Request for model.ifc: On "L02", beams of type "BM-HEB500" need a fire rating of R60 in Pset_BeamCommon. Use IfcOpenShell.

First a look at what the model holds.

```python
import ifcopenshell
import ifcopenshell.util.element

model = ifcopenshell.open("model.ifc")
print(model.schema)
storey = next(s for s in model.by_type("IfcBuildingStorey") if s.Name == "L02")
beams = [e for e in ifcopenshell.util.element.get_decomposition(storey) if e.is_a("IfcBeam")]
seen = {}
for e in beams:
    element_type = ifcopenshell.util.element.get_type(e)
    key = (element_type.Name if element_type != e and element_type else None, ifcopenshell.util.element.get_pset(e, "Pset_BeamCommon", "FireRating"))
    seen[key] = seen.get(key, 0) + 1
for (name, value), count in sorted(seen.items(), key=str):
    print(count, "x", name, "|", value)
```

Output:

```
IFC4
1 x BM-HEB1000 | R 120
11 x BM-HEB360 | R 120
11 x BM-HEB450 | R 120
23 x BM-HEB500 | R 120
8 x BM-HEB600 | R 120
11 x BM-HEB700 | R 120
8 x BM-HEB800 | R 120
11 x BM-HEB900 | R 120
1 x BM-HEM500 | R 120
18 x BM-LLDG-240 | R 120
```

```python
import ifcopenshell
import ifcopenshell.api.pset
import ifcopenshell.util.element

model = ifcopenshell.open("model.ifc")

storey = next(s for s in model.by_type("IfcBuildingStorey") if s.Name == "L02")
beams = [e for e in ifcopenshell.util.element.get_decomposition(storey) if e.is_a("IfcBeam")]

count = 0
for e in beams:
    element_type = ifcopenshell.util.element.get_type(e)
    if element_type in (None, e) or element_type.Name != "BM-HEB500":
        continue
    found = ifcopenshell.util.element.get_pset(e, "Pset_BeamCommon", should_inherit=False)
    if found:
        pset = model.by_id(found["id"])
        if len(ifcopenshell.util.element.get_elements_by_pset(pset)) > 1:
            pset = ifcopenshell.api.pset.unshare_pset(model, products=[e], pset=pset)[0]
    else:
        pset = ifcopenshell.api.pset.add_pset(model, product=e, name="Pset_BeamCommon")
    ifcopenshell.api.pset.edit_pset(model, pset=pset, properties={"FireRating": "R60"})
    count += 1

print(count, "beams updated")

model.write("model_v2.ifc")
```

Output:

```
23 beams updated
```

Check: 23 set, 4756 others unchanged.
